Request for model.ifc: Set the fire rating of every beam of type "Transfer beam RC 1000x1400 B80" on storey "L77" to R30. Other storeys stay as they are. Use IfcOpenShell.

First a look at what the model holds.

```python
import ifcopenshell
import ifcopenshell.util.element

model = ifcopenshell.open("model.ifc")
print(model.schema)
storey = next(s for s in model.by_type("IfcBuildingStorey") if s.Name == "L77")
beams = [e for e in ifcopenshell.util.element.get_decomposition(storey) if e.is_a("IfcBeam")]
seen = {}
for e in beams:
    element_type = ifcopenshell.util.element.get_type(e)
    key = (element_type.Name if element_type != e and element_type else None, ifcopenshell.util.element.get_pset(e, "Pset_BeamCommon", "FireRating"))
    seen[key] = seen.get(key, 0) + 1
for (name, value), count in sorted(seen.items(), key=str):
    print(count, "x", name, "|", value)
```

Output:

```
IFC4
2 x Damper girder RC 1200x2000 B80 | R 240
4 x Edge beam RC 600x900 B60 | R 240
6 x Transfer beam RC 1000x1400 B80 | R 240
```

```python
import ifcopenshell
import ifcopenshell.api.pset
import ifcopenshell.util.element

model = ifcopenshell.open("model.ifc")

storey = next(s for s in model.by_type("IfcBuildingStorey") if s.Name == "L77")
beams = [e for e in ifcopenshell.util.element.get_decomposition(storey) if e.is_a("IfcBeam")]

count = 0
for e in beams:
    element_type = ifcopenshell.util.element.get_type(e)
    if element_type in (None, e) or element_type.Name != "Transfer beam RC 1000x1400 B80":
        continue
    found = ifcopenshell.util.element.get_pset(e, "Pset_BeamCommon", should_inherit=False)
    if found:
        pset = model.by_id(found["id"])
        if len(ifcopenshell.util.element.get_elements_by_pset(pset)) > 1:
            pset = ifcopenshell.api.pset.unshare_pset(model, products=[e], pset=pset)[0]
    else:
        pset = ifcopenshell.api.pset.add_pset(model, product=e, name="Pset_BeamCommon")
    ifcopenshell.api.pset.edit_pset(model, pset=pset, properties={"FireRating": "R30"})
    count += 1

print(count, "beams updated")

model.write("model_updated.ifc")
```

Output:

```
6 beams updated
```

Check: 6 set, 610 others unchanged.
